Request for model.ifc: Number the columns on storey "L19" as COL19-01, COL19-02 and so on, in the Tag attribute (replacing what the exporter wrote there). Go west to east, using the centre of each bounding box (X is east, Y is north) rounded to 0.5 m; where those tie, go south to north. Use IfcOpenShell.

First a look at what the model holds.

```python
import ifcopenshell
import ifcopenshell.util.element
import ifcopenshell.util.placement

model = ifcopenshell.open("model.ifc")
print(model.schema)
storey = next(s for s in model.by_type("IfcBuildingStorey") if s.Name == "L19")
columns = [e for e in ifcopenshell.util.element.get_decomposition(storey) if e.is_a("IfcColumn")]
for e in sorted(columns, key=lambda e: e.id()):
    origin = ifcopenshell.util.placement.get_local_placement(e.ObjectPlacement)[:3, 3]
    print(e.id(), e.Tag, e.Name, origin.round(2) + 0.0, sep=" | ")
```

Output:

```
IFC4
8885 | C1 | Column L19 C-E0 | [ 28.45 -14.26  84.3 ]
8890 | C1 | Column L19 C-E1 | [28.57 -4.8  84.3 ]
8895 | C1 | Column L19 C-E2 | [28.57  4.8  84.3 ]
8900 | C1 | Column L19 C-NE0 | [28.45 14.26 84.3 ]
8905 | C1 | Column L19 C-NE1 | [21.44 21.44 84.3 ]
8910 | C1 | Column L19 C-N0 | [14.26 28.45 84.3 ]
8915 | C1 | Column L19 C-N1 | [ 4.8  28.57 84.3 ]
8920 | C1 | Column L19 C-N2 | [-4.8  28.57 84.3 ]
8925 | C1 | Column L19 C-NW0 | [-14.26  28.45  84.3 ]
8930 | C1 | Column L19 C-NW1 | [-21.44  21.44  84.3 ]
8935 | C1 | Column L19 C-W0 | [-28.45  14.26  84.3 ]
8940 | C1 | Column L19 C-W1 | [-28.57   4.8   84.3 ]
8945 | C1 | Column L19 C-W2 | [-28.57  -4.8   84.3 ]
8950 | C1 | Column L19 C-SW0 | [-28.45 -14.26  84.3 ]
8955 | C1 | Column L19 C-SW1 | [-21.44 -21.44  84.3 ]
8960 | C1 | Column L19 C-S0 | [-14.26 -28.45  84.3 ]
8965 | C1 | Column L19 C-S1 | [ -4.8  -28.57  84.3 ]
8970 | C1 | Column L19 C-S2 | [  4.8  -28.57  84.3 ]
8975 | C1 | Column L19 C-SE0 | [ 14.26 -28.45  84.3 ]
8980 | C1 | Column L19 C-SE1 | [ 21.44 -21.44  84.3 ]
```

```python
import ifcopenshell
import ifcopenshell.geom
import ifcopenshell.util.element
import ifcopenshell.util.shape

model = ifcopenshell.open("model.ifc")
settings = ifcopenshell.geom.settings()
settings.set("use-world-coords", True)


def centre(element):
    shape = ifcopenshell.geom.create_shape(settings, element)
    return ifcopenshell.util.shape.get_bbox_centroid(shape.geometry)


storey = next(s for s in model.by_type("IfcBuildingStorey") if s.Name == "L19")
columns = [e for e in ifcopenshell.util.element.get_decomposition(storey) if e.is_a("IfcColumn")]

# Insertion points can sit at a corner or the storey origin, so sort by the geometry (in metres).
centres = {e: centre(e) for e in columns}
columns.sort(key=lambda e: (round(centres[e][0] / 0.5), centres[e][1]))

for i, e in enumerate(columns, start=1):
    number = f"COL19-{i:02d}"
    e.Tag = number
    print(e.id(), number)

model.write("model_rev.ifc")
```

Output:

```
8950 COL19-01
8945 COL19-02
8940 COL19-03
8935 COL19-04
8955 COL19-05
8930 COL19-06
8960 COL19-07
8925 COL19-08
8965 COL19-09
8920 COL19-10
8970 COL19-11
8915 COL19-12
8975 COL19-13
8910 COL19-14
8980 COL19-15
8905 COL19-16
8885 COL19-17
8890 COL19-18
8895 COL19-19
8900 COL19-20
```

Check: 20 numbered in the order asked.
